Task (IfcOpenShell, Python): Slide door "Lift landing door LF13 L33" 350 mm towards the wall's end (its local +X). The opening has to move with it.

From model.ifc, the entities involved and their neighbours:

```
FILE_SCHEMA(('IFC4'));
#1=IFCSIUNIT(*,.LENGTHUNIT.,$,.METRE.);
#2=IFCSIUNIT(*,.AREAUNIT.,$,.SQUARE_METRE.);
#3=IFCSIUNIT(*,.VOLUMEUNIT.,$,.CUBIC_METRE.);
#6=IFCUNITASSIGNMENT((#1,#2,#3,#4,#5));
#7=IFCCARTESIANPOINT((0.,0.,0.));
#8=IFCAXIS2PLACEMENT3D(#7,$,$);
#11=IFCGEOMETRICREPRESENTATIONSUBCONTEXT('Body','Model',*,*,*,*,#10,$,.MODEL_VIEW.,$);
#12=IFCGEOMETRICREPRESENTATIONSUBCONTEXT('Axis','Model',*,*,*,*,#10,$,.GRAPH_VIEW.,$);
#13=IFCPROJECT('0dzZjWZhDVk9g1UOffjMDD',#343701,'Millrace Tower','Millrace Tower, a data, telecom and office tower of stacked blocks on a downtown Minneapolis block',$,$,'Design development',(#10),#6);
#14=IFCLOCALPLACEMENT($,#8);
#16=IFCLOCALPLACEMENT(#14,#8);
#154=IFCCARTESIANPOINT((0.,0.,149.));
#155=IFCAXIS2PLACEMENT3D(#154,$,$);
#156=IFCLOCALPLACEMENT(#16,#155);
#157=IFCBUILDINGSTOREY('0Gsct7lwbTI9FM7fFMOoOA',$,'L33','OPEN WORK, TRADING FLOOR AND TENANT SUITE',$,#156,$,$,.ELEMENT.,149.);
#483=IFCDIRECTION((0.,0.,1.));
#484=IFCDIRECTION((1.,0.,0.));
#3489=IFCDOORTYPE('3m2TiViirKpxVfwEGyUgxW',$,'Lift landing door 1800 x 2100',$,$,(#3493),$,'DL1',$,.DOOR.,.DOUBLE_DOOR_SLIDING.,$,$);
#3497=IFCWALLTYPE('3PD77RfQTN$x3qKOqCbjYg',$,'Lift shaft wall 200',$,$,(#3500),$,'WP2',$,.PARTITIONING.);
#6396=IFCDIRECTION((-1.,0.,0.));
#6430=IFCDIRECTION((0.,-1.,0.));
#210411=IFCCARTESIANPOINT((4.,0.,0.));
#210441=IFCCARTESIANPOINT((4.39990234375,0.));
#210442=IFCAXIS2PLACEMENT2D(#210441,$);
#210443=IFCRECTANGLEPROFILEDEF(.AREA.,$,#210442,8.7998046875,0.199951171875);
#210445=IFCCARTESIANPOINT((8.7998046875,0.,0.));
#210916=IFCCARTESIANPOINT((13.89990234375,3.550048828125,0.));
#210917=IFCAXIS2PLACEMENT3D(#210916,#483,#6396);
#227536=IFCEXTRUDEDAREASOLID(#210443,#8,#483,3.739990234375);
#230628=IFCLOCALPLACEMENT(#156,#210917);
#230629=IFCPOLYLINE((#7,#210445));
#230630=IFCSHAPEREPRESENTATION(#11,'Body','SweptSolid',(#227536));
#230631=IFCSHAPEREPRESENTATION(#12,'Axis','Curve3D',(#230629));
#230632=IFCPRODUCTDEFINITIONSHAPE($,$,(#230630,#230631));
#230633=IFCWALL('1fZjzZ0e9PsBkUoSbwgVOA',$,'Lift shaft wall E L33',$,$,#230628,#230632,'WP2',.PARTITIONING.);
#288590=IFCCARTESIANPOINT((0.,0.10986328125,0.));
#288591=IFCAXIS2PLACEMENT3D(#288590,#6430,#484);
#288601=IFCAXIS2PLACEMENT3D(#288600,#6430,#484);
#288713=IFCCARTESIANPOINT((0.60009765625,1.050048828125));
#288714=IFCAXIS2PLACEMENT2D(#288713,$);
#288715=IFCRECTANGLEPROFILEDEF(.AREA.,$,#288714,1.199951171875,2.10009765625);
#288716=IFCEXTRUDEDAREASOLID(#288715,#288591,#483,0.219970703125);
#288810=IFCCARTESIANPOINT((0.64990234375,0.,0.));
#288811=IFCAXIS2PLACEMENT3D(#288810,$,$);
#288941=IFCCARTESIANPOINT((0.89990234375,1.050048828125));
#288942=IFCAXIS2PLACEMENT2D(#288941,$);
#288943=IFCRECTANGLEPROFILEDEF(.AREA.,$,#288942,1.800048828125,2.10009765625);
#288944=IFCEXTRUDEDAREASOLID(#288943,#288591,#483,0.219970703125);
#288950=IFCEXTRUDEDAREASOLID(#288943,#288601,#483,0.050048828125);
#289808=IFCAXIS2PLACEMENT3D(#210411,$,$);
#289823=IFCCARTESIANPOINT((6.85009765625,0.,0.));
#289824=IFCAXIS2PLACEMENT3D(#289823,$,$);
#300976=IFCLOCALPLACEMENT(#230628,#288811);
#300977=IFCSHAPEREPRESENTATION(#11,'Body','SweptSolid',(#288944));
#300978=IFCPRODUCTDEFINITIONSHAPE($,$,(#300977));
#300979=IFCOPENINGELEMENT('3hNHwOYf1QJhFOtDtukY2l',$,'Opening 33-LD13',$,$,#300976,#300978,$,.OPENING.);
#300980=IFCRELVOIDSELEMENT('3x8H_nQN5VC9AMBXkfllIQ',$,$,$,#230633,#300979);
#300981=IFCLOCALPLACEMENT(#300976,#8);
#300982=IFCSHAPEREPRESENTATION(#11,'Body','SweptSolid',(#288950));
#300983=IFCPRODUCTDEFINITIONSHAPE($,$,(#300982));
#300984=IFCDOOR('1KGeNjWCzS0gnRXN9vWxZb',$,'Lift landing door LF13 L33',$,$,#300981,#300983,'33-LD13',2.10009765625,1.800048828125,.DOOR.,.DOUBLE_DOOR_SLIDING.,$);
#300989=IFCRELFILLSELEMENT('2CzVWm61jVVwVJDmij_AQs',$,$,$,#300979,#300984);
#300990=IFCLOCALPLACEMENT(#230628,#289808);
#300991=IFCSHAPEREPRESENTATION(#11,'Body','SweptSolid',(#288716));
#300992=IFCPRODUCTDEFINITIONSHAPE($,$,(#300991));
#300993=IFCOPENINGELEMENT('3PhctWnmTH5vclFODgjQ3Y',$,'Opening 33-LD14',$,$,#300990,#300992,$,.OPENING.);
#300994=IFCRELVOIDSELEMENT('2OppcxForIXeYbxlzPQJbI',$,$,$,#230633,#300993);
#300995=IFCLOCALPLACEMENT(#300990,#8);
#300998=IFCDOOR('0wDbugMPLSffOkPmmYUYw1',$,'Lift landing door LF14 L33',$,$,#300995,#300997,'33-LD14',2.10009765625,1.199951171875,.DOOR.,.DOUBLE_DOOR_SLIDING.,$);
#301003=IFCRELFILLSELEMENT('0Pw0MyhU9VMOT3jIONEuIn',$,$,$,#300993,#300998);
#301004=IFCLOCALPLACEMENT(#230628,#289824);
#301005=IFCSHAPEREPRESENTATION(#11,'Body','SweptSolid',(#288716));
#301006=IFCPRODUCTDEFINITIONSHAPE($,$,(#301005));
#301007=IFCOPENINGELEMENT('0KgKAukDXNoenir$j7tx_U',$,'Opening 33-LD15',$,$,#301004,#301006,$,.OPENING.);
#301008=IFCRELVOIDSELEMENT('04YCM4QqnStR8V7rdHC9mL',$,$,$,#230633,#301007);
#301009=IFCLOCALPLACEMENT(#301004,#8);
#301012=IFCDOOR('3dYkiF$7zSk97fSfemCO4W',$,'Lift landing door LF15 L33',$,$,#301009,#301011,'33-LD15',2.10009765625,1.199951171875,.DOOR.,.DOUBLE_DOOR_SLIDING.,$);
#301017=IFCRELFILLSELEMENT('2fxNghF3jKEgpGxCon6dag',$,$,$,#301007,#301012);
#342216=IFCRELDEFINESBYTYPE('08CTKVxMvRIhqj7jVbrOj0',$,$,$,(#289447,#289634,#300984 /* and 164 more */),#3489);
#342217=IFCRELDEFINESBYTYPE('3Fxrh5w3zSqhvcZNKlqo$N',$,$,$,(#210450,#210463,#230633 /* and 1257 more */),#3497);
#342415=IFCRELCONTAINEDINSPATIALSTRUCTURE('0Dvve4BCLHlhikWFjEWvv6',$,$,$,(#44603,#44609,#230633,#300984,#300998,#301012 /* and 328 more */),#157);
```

```python
import ifcopenshell
import ifcopenshell.api.geometry
import ifcopenshell.util.placement
import ifcopenshell.util.unit

model = ifcopenshell.open("model.ifc")
unit_scale = ifcopenshell.util.unit.calculate_unit_scale(model)

door = model.by_guid("1KGeNjWCzS0gnRXN9vWxZb")
opening = door.FillsVoids[0].RelatingOpeningElement
wall = opening.VoidsElements[0].RelatingBuildingElement

wall_matrix = ifcopenshell.util.placement.get_local_placement(wall.ObjectPlacement)
shift = wall_matrix[:3, 0] * 0.35 / unit_scale
before = ifcopenshell.util.placement.get_local_placement(door.ObjectPlacement)[:3, 3].copy()

# The door is placed relative to its opening, so it follows when the opening moves.
matrix = ifcopenshell.util.placement.get_local_placement(opening.ObjectPlacement)
matrix[:3, 3] += shift
ifcopenshell.api.geometry.edit_object_placement(
    model, product=opening, matrix=matrix, is_si=False, should_transform_children=True
)

after = ifcopenshell.util.placement.get_local_placement(door.ObjectPlacement)[:3, 3]
print("door moved by", (after - before).round(3) + 0.0)

model.write("model-out.ifc")
```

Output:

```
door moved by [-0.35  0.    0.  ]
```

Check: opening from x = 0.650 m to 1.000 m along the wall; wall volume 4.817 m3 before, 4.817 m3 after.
